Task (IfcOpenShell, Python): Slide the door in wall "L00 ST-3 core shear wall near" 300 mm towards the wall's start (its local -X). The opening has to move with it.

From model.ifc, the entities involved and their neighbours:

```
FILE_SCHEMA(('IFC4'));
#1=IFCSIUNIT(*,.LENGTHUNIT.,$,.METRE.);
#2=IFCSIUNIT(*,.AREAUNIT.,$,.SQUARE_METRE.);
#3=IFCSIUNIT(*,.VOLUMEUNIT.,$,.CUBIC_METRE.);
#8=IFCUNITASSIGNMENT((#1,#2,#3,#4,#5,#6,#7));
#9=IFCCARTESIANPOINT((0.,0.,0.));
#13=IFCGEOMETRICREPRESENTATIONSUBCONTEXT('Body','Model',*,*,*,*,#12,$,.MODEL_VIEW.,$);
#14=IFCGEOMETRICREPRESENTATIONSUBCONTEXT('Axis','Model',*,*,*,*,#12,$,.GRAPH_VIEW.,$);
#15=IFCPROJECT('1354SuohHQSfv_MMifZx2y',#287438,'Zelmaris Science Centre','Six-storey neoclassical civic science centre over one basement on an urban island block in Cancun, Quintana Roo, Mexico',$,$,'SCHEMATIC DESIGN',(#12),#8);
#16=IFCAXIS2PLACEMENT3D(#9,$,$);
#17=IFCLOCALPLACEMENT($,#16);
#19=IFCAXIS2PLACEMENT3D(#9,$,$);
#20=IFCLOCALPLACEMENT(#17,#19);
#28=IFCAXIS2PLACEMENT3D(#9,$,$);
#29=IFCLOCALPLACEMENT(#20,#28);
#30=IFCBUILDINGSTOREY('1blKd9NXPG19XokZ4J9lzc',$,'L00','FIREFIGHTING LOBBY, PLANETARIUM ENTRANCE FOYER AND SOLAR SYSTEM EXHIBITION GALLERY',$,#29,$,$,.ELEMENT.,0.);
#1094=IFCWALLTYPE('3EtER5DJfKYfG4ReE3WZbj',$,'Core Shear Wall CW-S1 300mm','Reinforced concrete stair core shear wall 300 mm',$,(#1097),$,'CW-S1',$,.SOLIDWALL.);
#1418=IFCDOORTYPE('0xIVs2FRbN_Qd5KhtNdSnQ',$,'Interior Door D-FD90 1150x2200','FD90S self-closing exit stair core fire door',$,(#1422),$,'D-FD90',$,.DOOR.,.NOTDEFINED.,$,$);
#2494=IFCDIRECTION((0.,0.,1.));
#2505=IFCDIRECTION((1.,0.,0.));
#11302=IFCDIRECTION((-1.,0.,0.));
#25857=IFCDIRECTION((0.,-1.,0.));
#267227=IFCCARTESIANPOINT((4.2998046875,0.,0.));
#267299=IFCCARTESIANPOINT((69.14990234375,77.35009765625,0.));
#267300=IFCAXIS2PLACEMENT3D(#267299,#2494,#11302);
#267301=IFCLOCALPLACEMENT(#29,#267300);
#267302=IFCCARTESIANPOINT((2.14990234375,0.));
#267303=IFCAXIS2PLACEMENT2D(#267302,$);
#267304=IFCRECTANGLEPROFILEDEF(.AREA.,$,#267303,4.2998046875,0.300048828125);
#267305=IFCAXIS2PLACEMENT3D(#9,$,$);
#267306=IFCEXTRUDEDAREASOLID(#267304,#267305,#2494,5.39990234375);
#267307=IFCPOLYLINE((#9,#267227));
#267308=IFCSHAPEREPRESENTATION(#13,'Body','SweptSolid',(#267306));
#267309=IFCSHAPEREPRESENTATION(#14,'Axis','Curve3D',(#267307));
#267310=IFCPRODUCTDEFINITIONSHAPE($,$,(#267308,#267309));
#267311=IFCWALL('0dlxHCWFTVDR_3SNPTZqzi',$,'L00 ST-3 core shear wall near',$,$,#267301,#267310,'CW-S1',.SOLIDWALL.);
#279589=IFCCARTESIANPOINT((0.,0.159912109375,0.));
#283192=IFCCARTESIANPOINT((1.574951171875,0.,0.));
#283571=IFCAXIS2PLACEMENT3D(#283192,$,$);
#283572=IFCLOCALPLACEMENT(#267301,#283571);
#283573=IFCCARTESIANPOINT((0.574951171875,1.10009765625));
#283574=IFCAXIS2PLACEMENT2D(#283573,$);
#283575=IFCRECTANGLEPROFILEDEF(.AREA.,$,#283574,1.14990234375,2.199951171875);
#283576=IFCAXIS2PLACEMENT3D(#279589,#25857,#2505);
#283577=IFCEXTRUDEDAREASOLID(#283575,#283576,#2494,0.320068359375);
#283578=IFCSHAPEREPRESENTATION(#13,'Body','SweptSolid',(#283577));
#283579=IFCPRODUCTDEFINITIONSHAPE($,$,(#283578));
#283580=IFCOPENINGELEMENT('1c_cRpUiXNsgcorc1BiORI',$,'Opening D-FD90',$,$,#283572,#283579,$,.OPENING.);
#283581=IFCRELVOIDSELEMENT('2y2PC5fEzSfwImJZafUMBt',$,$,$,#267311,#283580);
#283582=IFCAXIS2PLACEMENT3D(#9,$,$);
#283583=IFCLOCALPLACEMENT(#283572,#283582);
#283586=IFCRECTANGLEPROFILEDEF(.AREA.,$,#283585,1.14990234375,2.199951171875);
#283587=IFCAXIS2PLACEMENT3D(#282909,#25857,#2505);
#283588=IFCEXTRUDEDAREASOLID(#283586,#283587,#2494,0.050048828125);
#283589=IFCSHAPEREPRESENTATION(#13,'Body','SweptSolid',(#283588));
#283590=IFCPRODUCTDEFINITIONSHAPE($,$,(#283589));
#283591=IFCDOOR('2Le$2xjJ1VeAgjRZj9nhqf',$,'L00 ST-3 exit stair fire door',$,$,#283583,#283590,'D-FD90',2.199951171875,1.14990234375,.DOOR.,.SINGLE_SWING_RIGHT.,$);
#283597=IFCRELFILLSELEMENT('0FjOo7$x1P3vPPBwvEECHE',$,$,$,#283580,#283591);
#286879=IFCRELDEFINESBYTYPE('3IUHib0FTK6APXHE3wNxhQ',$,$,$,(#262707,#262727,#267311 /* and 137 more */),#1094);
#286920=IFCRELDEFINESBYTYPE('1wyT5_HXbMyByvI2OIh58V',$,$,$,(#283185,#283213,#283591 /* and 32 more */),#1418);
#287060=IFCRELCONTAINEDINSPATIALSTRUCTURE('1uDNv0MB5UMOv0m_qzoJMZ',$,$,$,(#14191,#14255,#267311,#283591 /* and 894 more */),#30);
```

```python
import ifcopenshell
import ifcopenshell.api.geometry
import ifcopenshell.util.placement
import ifcopenshell.util.unit

model = ifcopenshell.open("model.ifc")
unit_scale = ifcopenshell.util.unit.calculate_unit_scale(model)

door = model.by_guid("2Le$2xjJ1VeAgjRZj9nhqf")
opening = door.FillsVoids[0].RelatingOpeningElement
wall = opening.VoidsElements[0].RelatingBuildingElement

wall_matrix = ifcopenshell.util.placement.get_local_placement(wall.ObjectPlacement)
shift = wall_matrix[:3, 0] * -0.3 / unit_scale
before = ifcopenshell.util.placement.get_local_placement(door.ObjectPlacement)[:3, 3].copy()

# The door is placed relative to its opening, so it follows when the opening moves.
matrix = ifcopenshell.util.placement.get_local_placement(opening.ObjectPlacement)
matrix[:3, 3] += shift
ifcopenshell.api.geometry.edit_object_placement(
    model, product=opening, matrix=matrix, is_si=False, should_transform_children=True
)

after = ifcopenshell.util.placement.get_local_placement(door.ObjectPlacement)[:3, 3]
print("door moved by", (after - before).round(3) + 0.0)

model.write("model_v2.ifc")
```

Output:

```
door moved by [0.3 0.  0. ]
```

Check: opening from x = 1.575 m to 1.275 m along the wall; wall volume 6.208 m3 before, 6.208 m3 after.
